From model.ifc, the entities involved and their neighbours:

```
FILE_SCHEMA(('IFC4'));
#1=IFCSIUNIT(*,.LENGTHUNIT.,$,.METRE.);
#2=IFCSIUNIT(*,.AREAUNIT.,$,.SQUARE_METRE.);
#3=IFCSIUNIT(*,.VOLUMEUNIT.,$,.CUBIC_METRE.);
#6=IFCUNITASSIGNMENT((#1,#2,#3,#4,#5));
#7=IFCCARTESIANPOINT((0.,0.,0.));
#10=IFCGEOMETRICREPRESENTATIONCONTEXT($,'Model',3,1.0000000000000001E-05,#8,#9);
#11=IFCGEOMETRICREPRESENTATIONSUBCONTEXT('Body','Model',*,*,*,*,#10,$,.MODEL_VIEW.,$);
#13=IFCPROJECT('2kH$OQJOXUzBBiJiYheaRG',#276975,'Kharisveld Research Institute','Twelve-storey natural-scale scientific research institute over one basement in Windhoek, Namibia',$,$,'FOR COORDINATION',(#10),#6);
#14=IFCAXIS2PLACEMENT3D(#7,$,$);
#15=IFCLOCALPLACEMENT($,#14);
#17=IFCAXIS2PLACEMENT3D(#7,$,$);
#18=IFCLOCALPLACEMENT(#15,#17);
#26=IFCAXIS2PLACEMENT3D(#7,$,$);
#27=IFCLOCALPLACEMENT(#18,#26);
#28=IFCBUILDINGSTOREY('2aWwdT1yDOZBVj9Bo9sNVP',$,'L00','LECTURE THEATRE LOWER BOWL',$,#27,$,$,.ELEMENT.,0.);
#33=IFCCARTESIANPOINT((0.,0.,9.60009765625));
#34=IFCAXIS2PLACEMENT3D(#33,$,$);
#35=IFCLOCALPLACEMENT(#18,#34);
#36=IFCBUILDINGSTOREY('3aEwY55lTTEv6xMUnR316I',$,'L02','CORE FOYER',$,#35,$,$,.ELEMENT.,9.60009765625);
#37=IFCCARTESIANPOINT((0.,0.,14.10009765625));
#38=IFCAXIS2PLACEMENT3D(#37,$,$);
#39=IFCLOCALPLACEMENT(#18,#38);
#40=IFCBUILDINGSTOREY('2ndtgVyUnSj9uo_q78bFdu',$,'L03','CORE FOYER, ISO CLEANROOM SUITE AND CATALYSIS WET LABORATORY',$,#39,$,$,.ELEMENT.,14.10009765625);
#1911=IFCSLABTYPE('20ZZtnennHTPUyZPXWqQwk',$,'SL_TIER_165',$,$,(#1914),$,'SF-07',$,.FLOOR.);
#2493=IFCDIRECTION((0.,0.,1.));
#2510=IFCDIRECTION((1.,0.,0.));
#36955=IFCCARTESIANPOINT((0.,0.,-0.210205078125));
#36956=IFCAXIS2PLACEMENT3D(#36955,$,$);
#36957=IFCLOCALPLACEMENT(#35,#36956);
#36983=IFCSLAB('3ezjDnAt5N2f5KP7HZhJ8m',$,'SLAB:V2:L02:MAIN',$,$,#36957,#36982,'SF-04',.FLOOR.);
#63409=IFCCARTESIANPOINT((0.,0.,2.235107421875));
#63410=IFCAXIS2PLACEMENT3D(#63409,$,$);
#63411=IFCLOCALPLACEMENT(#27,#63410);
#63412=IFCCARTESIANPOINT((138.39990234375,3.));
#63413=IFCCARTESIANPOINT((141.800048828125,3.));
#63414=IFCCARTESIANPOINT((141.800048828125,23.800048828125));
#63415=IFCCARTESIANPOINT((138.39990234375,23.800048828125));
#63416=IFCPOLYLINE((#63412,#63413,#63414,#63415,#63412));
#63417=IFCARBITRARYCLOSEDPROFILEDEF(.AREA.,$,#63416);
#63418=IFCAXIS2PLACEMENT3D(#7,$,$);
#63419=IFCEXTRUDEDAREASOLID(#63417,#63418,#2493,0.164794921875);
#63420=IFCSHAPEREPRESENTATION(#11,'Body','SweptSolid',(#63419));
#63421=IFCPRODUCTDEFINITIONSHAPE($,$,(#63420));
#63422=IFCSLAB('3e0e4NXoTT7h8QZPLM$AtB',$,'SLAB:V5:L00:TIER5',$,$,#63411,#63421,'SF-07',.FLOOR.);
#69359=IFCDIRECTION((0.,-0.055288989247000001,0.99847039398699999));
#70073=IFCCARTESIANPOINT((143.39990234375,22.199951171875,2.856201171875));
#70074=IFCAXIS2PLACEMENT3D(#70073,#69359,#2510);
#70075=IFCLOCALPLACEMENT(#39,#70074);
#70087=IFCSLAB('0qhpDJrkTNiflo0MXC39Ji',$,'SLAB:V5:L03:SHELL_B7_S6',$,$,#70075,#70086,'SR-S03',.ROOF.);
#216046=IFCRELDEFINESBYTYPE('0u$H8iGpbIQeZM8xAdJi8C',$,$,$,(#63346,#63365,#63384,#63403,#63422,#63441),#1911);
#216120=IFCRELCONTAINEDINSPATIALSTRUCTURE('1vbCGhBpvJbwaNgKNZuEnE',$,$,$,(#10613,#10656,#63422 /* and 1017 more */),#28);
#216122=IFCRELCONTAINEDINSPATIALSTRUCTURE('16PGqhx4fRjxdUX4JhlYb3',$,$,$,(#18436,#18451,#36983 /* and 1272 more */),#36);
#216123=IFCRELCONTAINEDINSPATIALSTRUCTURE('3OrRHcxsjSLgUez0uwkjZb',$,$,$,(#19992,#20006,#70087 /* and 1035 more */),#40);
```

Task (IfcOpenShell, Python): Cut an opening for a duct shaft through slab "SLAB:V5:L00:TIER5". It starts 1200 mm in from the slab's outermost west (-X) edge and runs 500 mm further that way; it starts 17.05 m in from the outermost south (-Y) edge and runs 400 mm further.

```python
import numpy as np
import ifcopenshell
import ifcopenshell.api.feature
import ifcopenshell.api.geometry
import ifcopenshell.api.root
import ifcopenshell.geom
import ifcopenshell.util.placement
import ifcopenshell.util.representation
import ifcopenshell.util.shape
import ifcopenshell.util.unit

model = ifcopenshell.open("model.ifc")
unit_scale = ifcopenshell.util.unit.calculate_unit_scale(model)
settings = ifcopenshell.geom.settings()


def volume(element):
    """Net volume in cubic metres, openings subtracted."""
    shape = ifcopenshell.geom.create_shape(settings, element)
    return ifcopenshell.util.shape.get_volume(shape.geometry)


slab = model.by_guid("3e0e4NXoTT7h8QZPLM$AtB")
before = volume(slab)

# Extent in the slab's own axes, in metres. The edges named are its -X and -Y sides.
slab_shape = ifcopenshell.geom.create_shape(settings, slab)
vertices = ifcopenshell.util.shape.get_vertices(slab_shape.geometry)
x_min, y_min, bottom = vertices.min(axis=0)
top = vertices[:, 2].max()

opening = ifcopenshell.api.root.create_entity(model, ifc_class="IfcOpeningElement", name="Duct shaft opening", predefined_type="OPENING")
context = ifcopenshell.util.representation.get_context(model, "Model", "Body", "MODEL_VIEW")
width, depth = 0.5, 0.4
outline = [(0.0, 0.0), (width, 0.0), (width, depth), (0.0, depth), (0.0, 0.0)]
# Overshoot both faces by 50 mm so the cut is clean.
shape = ifcopenshell.api.geometry.add_slab_representation(
    model, context=context, depth=top - bottom + 0.1, polyline=outline
)
ifcopenshell.api.geometry.assign_representation(model, product=opening, representation=shape)

matrix = ifcopenshell.util.placement.get_local_placement(slab.ObjectPlacement)
matrix[:, 3] = matrix @ np.append(np.array([x_min + 1.2, y_min + 17.05, bottom - 0.05]) / unit_scale, 1.0)
ifcopenshell.api.geometry.edit_object_placement(model, product=opening, matrix=matrix, is_si=False)
ifcopenshell.api.feature.add_feature(model, feature=opening, element=slab)

after = volume(slab)

print(f"slab volume {before:.3f} -> {after:.3f} m3")

model.write("model_updated.ifc")
```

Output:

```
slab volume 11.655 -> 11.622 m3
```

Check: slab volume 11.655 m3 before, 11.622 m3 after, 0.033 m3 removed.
